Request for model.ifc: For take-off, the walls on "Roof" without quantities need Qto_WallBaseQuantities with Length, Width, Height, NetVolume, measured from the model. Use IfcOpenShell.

First a look at what the model holds.

```python
import ifcopenshell
import ifcopenshell.util.element
import ifcopenshell.util.unit

model = ifcopenshell.open("model.ifc")
print(model.schema)
for unit_type in ("LENGTHUNIT", "AREAUNIT", "VOLUMEUNIT"):
    print(unit_type, ifcopenshell.util.unit.calculate_unit_scale(model, unit_type))
storey = next(s for s in model.by_type("IfcBuildingStorey") if s.Name == "Roof")
walls = [e for e in ifcopenshell.util.element.get_decomposition(storey) if e.is_a("IfcWall")]
for e in sorted(walls, key=lambda e: e.id()):
    print(e.id(), e.is_a(), e.Name, list(ifcopenshell.util.element.get_psets(e, qtos_only=True)), sep=" | ")
```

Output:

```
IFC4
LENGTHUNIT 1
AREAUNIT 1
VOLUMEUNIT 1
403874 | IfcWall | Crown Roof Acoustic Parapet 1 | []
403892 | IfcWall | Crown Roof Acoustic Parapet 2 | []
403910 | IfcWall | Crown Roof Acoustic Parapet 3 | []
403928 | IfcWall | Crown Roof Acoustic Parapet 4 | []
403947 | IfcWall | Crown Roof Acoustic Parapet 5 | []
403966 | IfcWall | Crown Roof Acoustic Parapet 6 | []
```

```python
import ifcopenshell
import ifcopenshell.api.pset
import ifcopenshell.geom
import ifcopenshell.util.element
import ifcopenshell.util.shape
import ifcopenshell.util.unit

model = ifcopenshell.open("model.ifc")
unit_scale = ifcopenshell.util.unit.calculate_unit_scale(model)
volume_scale = ifcopenshell.util.unit.calculate_unit_scale(model, "VOLUMEUNIT")
settings = ifcopenshell.geom.settings()

storey = next(s for s in model.by_type("IfcBuildingStorey") if s.Name == "Roof")
walls = [e for e in ifcopenshell.util.element.get_decomposition(storey) if e.is_a("IfcWall")]

for e in sorted(walls, key=lambda e: e.id()):
    if ifcopenshell.util.element.get_psets(e, qtos_only=True, should_inherit=False):
        continue
    # Geometry comes back in metres, in the element's own axes.
    shape = ifcopenshell.geom.create_shape(settings, e)
    values = {
        "Length": ifcopenshell.util.shape.get_x(shape.geometry) / unit_scale,
        "Width": ifcopenshell.util.shape.get_y(shape.geometry) / unit_scale,
        "Height": ifcopenshell.util.shape.get_z(shape.geometry) / unit_scale,
        "NetVolume": ifcopenshell.util.shape.get_volume(shape.geometry) / volume_scale,
    }
    qto = ifcopenshell.api.pset.add_qto(model, product=e, name="Qto_WallBaseQuantities")
    ifcopenshell.api.pset.edit_qto(model, qto=qto, properties=values)
    print(e.id(), {k: round(v, 3) for k, v in values.items()})

model.write("model_rev.ifc")
```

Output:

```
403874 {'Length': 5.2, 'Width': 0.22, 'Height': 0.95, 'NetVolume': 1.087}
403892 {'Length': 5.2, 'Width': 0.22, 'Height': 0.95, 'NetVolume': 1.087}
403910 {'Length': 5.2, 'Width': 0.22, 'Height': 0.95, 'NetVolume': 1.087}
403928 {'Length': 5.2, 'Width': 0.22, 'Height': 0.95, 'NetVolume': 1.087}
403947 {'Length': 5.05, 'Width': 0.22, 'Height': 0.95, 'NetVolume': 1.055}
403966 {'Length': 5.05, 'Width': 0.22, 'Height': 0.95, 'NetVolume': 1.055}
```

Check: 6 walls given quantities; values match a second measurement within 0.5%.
